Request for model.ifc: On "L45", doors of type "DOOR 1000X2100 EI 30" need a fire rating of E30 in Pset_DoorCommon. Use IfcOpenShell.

First a look at what the model holds.

```python
import ifcopenshell
import ifcopenshell.util.element

model = ifcopenshell.open("model.ifc")
print(model.schema)
storey = next(s for s in model.by_type("IfcBuildingStorey") if s.Name == "L45")
doors = [e for e in ifcopenshell.util.element.get_decomposition(storey) if e.is_a("IfcDoor")]
seen = {}
for e in doors:
    element_type = ifcopenshell.util.element.get_type(e)
    key = (element_type.Name if element_type != e and element_type else None, ifcopenshell.util.element.get_pset(e, "Pset_DoorCommon", "FireRating"))
    seen[key] = seen.get(key, 0) + 1
for (name, value), count in sorted(seen.items(), key=str):
    print(count, "x", name, "|", value)
```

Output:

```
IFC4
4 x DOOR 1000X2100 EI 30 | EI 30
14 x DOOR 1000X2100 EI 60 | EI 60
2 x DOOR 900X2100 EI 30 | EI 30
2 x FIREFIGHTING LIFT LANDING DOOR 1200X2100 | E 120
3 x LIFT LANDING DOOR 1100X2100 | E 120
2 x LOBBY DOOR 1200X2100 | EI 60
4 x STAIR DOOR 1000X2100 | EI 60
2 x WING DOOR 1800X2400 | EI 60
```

```python
import ifcopenshell
import ifcopenshell.api.pset
import ifcopenshell.util.element

model = ifcopenshell.open("model.ifc")

storey = next(s for s in model.by_type("IfcBuildingStorey") if s.Name == "L45")
doors = [e for e in ifcopenshell.util.element.get_decomposition(storey) if e.is_a("IfcDoor")]

count = 0
for e in doors:
    element_type = ifcopenshell.util.element.get_type(e)
    if element_type in (None, e) or element_type.Name != "DOOR 1000X2100 EI 30":
        continue
    found = ifcopenshell.util.element.get_pset(e, "Pset_DoorCommon", should_inherit=False)
    if found:
        pset = model.by_id(found["id"])
        if len(ifcopenshell.util.element.get_elements_by_pset(pset)) > 1:
            pset = ifcopenshell.api.pset.unshare_pset(model, products=[e], pset=pset)[0]
    else:
        pset = ifcopenshell.api.pset.add_pset(model, product=e, name="Pset_DoorCommon")
    ifcopenshell.api.pset.edit_pset(model, pset=pset, properties={"FireRating": "E30"})
    count += 1

print(count, "doors updated")

model.write("model_updated.ifc")
```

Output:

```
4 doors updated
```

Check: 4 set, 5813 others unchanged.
